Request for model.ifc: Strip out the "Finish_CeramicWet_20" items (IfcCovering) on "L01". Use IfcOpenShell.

First a look at what the model holds.

```python
import ifcopenshell
import ifcopenshell.util.element

model = ifcopenshell.open("model.ifc")
print(model.schema)
storey = next(s for s in model.by_type("IfcBuildingStorey") if s.Name == "L01")
coverings = [e for e in ifcopenshell.util.element.get_decomposition(storey) if e.is_a("IfcCovering")]
seen = {}
for e in coverings:
    element_type = ifcopenshell.util.element.get_type(e)
    name = element_type.Name if element_type not in (None, e) else None
    seen[name] = seen.get(name, 0) + 1
for name, count in sorted(seen.items(), key=str):
    print(count, "x", name)
```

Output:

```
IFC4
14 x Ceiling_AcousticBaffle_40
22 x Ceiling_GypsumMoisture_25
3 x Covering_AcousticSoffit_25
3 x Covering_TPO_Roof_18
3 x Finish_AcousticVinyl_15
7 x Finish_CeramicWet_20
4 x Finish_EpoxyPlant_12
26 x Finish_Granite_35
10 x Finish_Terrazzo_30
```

```python
import ifcopenshell
import ifcopenshell.api.root
import ifcopenshell.util.element

model = ifcopenshell.open("model.ifc")

storey = next(s for s in model.by_type("IfcBuildingStorey") if s.Name == "L01")
coverings = [e for e in ifcopenshell.util.element.get_decomposition(storey) if e.is_a("IfcCovering")]
targets = [e for e in coverings if (t := ifcopenshell.util.element.get_type(e)) not in (None, e) and t.Name == "Finish_CeramicWet_20"]

for e in targets:
    ifcopenshell.api.root.remove_product(model, product=e)
print(len(targets), "removed")

model.write("model_rev.ifc")
```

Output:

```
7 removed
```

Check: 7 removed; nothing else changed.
